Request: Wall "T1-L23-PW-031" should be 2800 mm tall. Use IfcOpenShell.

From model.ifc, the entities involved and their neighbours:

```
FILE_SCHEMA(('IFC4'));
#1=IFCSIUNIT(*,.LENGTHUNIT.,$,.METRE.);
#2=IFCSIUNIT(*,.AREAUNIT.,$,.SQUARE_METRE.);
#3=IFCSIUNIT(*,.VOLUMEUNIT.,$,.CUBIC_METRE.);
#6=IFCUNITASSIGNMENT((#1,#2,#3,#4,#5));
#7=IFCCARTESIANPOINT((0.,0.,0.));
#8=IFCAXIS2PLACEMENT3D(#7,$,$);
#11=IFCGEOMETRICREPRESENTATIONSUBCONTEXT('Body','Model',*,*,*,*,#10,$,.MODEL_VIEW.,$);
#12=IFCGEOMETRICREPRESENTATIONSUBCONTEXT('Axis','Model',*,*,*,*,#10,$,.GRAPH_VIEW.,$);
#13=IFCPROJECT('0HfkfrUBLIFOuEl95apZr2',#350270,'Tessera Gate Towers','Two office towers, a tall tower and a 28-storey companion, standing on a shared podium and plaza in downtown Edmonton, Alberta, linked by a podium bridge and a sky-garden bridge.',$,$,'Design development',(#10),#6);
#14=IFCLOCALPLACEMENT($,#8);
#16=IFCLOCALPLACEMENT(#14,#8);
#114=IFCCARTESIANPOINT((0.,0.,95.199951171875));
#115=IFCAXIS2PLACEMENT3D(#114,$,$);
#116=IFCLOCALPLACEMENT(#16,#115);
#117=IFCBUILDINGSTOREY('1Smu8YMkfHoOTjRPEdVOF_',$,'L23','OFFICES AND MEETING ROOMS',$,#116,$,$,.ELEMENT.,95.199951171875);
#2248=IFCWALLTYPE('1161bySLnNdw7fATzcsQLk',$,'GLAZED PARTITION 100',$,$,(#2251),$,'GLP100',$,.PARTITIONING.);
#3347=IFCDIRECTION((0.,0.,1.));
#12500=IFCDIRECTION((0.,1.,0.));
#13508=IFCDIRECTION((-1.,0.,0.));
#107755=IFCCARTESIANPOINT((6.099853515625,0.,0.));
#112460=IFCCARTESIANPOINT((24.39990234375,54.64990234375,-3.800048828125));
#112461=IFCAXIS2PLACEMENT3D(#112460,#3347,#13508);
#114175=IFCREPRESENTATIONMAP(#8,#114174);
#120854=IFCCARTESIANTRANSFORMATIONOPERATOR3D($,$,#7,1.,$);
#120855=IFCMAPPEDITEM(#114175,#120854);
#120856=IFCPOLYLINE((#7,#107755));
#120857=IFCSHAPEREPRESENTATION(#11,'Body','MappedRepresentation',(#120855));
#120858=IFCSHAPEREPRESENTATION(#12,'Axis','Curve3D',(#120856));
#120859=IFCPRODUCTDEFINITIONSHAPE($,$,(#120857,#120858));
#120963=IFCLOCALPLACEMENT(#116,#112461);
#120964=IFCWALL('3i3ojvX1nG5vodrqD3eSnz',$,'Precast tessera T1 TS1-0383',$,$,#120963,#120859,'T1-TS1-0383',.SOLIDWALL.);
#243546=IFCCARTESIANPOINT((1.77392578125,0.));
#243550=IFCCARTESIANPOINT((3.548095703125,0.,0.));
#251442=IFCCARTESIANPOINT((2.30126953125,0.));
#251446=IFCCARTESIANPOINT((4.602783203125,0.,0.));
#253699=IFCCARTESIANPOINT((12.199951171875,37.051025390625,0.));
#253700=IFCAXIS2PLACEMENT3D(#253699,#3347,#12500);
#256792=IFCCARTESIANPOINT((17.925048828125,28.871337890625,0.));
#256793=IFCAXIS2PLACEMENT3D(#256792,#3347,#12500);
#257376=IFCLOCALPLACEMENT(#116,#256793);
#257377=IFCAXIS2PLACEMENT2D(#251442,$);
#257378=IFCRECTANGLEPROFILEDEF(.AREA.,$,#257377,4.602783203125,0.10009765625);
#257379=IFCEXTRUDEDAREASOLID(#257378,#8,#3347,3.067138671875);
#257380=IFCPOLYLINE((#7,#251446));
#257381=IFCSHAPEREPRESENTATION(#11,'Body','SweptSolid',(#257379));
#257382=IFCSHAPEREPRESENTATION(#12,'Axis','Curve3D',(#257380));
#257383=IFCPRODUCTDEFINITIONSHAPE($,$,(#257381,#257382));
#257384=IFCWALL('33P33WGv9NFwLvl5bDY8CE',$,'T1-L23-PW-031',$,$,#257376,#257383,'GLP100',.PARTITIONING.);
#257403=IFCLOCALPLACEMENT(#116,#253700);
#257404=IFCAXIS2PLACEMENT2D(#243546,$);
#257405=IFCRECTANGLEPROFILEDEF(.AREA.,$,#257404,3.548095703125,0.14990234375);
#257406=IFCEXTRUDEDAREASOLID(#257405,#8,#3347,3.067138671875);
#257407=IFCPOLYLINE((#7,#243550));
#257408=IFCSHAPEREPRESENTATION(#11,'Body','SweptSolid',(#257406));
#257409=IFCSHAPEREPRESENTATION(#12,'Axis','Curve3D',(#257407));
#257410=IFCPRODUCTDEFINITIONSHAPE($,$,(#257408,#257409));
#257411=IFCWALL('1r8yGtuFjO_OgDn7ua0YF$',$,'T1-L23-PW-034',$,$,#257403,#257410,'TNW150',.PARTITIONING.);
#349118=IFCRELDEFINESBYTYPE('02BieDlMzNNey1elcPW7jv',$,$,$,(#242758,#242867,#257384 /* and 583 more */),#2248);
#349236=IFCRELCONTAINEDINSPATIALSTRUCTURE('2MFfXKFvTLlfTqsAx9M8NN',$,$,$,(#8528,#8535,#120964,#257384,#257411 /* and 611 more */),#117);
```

```python
import ifcopenshell
import ifcopenshell.geom
import ifcopenshell.util.representation
import ifcopenshell.util.shape

model = ifcopenshell.open("model.ifc")
settings = ifcopenshell.geom.settings()


def volume(element):
    """Net volume in cubic metres, openings subtracted."""
    shape = ifcopenshell.geom.create_shape(settings, element)
    return ifcopenshell.util.shape.get_volume(shape.geometry)


wall = model.by_id(257384)
before = volume(wall)

body = ifcopenshell.util.representation.get_representation(wall, "Model", "Body")
solid = body.Items[0]
old_height = solid.Depth
solid.Depth = 2.8
after = volume(wall)

print(f"height {old_height:g} -> {solid.Depth:g}, volume {before:.3f} -> {after:.3f} m3")

model.write("model-out.ifc")
```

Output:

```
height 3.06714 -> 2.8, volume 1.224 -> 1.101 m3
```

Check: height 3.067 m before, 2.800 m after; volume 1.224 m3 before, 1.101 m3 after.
